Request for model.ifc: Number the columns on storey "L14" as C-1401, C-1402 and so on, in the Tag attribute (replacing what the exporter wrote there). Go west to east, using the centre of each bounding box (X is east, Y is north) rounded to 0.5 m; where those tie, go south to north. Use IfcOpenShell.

First a look at what the model holds.

```python
import ifcopenshell
import ifcopenshell.util.element
import ifcopenshell.util.placement

model = ifcopenshell.open("model.ifc")
print(model.schema)
storey = next(s for s in model.by_type("IfcBuildingStorey") if s.Name == "L14")
columns = [e for e in ifcopenshell.util.element.get_decomposition(storey) if e.is_a("IfcColumn")]
for e in sorted(columns, key=lambda e: e.id()):
    origin = ifcopenshell.util.placement.get_local_placement(e.ObjectPlacement)[:3, 3]
    print(e.id(), e.Tag, e.Name, origin.round(2) + 0.0, sep=" | ")
```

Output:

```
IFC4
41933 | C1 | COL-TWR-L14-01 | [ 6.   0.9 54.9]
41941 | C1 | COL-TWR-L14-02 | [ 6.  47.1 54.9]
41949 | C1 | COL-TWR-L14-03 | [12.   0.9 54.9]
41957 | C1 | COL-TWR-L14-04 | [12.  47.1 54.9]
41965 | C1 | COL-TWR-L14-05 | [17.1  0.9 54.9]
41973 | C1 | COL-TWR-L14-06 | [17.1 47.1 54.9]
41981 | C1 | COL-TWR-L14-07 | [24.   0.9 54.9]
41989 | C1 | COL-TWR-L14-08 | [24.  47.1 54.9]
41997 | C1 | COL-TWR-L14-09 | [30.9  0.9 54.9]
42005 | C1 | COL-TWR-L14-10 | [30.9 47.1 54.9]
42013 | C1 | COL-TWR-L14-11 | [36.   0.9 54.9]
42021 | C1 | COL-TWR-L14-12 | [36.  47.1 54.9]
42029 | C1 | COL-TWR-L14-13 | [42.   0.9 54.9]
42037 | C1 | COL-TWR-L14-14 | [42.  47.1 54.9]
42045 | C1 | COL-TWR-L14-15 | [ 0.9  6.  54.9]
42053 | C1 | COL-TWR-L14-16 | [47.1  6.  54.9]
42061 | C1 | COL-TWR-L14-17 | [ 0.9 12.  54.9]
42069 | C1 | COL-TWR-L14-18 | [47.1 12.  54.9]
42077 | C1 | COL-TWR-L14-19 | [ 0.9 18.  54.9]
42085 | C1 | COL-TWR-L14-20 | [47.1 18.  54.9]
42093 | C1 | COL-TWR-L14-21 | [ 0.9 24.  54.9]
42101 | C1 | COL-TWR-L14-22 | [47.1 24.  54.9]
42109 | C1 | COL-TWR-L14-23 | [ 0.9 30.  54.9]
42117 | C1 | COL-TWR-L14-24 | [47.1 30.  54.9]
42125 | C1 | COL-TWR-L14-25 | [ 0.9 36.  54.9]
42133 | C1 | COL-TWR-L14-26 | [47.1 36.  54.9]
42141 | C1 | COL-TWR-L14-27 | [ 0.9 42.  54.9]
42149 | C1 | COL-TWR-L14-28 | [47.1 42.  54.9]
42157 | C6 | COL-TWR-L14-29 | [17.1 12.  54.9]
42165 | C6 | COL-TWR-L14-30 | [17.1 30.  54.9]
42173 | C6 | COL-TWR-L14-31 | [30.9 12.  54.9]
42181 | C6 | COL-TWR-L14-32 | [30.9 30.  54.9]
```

```python
import ifcopenshell
import ifcopenshell.geom
import ifcopenshell.util.element
import ifcopenshell.util.shape

model = ifcopenshell.open("model.ifc")
settings = ifcopenshell.geom.settings()
settings.set("use-world-coords", True)


def centre(element):
    shape = ifcopenshell.geom.create_shape(settings, element)
    return ifcopenshell.util.shape.get_bbox_centroid(shape.geometry)


storey = next(s for s in model.by_type("IfcBuildingStorey") if s.Name == "L14")
columns = [e for e in ifcopenshell.util.element.get_decomposition(storey) if e.is_a("IfcColumn")]

# Insertion points can sit at a corner or the storey origin, so sort by the geometry (in metres).
centres = {e: centre(e) for e in columns}
columns.sort(key=lambda e: (round(centres[e][0] / 0.5), centres[e][1]))

for i, e in enumerate(columns, start=1):
    number = f"C-14{i:02d}"
    e.Tag = number
    print(e.id(), number)

model.write("model-out.ifc")
```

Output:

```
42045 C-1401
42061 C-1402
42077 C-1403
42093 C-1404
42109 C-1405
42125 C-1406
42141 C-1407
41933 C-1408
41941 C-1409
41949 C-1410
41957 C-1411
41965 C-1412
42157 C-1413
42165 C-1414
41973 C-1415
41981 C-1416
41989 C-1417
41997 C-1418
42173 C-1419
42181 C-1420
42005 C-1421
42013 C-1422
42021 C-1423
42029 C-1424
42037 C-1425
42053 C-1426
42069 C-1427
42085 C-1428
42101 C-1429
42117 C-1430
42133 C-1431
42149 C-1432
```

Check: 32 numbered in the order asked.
